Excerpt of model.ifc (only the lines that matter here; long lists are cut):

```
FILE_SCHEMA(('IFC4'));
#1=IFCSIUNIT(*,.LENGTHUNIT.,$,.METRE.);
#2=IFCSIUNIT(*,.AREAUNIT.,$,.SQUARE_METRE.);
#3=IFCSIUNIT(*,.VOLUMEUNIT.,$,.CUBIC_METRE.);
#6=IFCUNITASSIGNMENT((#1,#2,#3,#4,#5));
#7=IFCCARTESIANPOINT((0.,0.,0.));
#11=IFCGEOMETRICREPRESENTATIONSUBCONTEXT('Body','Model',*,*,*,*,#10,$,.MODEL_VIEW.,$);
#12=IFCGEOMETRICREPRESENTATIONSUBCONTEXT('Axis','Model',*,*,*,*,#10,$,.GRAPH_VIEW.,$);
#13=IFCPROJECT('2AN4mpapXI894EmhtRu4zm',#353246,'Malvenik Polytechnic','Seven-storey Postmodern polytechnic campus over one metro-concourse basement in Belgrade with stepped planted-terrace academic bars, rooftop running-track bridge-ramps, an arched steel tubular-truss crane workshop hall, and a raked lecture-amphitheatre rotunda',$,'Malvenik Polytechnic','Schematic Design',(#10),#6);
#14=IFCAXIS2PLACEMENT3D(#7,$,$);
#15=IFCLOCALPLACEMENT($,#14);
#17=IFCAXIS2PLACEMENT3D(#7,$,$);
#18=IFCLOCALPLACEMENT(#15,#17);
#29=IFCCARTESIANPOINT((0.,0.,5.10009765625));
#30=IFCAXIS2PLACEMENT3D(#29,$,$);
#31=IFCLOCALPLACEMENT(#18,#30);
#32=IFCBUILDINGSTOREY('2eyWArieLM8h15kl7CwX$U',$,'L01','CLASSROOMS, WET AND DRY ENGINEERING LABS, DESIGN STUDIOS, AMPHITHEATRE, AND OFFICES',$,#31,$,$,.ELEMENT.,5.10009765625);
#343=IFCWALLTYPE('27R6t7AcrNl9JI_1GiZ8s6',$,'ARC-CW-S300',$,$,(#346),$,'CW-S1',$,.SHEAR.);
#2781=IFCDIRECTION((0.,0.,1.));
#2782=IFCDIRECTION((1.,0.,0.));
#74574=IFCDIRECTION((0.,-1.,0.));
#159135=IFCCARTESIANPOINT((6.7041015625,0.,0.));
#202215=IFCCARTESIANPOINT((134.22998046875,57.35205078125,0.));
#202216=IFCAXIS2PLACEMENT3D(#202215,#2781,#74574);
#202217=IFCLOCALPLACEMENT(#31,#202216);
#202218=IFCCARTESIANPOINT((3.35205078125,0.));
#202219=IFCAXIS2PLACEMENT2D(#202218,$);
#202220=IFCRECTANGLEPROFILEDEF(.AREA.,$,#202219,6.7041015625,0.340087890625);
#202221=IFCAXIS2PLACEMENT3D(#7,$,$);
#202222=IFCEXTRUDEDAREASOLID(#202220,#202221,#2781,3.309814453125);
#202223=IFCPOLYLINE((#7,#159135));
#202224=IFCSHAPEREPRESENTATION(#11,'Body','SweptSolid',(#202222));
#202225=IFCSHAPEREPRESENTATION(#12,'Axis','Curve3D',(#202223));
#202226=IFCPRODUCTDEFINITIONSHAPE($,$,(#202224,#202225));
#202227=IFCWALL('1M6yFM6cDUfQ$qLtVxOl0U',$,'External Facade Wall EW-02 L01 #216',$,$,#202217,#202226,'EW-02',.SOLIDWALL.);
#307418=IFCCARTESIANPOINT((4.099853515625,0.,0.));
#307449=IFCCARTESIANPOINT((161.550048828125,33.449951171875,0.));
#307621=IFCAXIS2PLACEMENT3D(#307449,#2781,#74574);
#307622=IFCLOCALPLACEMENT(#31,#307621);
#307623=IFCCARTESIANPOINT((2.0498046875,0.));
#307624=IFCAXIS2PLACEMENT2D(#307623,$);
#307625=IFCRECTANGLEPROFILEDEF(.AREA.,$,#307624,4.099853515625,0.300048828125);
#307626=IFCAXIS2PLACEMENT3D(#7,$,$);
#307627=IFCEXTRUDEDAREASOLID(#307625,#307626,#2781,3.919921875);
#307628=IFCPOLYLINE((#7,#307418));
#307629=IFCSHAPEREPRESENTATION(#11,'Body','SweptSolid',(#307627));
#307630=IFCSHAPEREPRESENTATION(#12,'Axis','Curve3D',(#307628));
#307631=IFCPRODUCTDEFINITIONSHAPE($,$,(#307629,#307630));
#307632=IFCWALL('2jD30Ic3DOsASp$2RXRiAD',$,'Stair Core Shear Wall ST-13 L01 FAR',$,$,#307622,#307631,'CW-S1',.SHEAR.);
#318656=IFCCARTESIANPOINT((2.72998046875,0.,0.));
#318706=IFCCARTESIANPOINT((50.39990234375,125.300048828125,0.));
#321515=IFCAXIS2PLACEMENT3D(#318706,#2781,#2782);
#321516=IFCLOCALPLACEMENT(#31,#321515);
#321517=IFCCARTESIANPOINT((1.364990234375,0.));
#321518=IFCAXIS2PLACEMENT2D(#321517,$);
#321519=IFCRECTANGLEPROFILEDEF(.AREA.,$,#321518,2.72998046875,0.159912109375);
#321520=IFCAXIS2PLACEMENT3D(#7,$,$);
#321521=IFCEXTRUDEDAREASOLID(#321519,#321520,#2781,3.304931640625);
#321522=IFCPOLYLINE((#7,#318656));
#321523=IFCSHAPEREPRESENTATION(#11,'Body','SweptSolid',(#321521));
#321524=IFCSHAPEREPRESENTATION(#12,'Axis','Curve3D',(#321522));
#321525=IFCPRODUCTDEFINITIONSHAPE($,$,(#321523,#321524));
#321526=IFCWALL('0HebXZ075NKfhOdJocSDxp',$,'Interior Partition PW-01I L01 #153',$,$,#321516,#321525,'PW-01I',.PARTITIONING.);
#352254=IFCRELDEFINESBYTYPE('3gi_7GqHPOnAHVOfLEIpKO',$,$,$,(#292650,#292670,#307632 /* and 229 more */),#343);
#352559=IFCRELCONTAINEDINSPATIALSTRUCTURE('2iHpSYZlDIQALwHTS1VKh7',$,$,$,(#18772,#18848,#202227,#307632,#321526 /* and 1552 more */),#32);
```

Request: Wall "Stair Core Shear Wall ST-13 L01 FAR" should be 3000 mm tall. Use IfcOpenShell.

```python
import ifcopenshell
import ifcopenshell.geom
import ifcopenshell.util.representation
import ifcopenshell.util.shape

model = ifcopenshell.open("model.ifc")
settings = ifcopenshell.geom.settings()


def volume(element):
    """Net volume in cubic metres, openings subtracted."""
    shape = ifcopenshell.geom.create_shape(settings, element)
    return ifcopenshell.util.shape.get_volume(shape.geometry)


wall = model.by_guid("2jD30Ic3DOsASp$2RXRiAD")
before = volume(wall)

body = ifcopenshell.util.representation.get_representation(wall, "Model", "Body")
solid = body.Items[0]
old_height = solid.Depth
solid.Depth = 3.0
after = volume(wall)

print(f"height {old_height:g} -> {solid.Depth:g}, volume {before:.3f} -> {after:.3f} m3")

model.write("model_updated.ifc")
```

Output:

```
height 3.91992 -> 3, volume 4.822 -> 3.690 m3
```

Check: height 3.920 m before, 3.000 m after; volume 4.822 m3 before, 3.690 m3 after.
